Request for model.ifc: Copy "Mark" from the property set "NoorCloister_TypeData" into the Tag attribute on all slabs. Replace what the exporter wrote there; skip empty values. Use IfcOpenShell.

First a look at what the model holds.

```python
import ifcopenshell
import ifcopenshell.util.element

model = ifcopenshell.open("model.ifc")
print(model.schema)
slabs = model.by_type("IfcSlab")
print(len(slabs), "slabs")
for e in slabs[:8]:
    source = ifcopenshell.util.element.get_pset(e, "NoorCloister_TypeData", "Mark")
    target = e.Tag
    print(e.id(), repr(source), repr(target), sep=" | ")
```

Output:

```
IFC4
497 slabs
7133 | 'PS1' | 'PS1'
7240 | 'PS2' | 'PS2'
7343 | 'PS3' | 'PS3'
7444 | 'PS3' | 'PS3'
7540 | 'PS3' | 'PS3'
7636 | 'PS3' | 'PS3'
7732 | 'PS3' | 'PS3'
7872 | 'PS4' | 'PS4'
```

```python
import ifcopenshell
import ifcopenshell.util.element

model = ifcopenshell.open("model.ifc")

count = 0
for e in model.by_type("IfcSlab"):
    value = ifcopenshell.util.element.get_pset(e, "NoorCloister_TypeData", "Mark")
    current = e.Tag
    if not value or not value.strip() or current == value:
        continue
    e.Tag = value
    count += 1

print(count, "slabs updated")

model.write("model_edited.ifc")
```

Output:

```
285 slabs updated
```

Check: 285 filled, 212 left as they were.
